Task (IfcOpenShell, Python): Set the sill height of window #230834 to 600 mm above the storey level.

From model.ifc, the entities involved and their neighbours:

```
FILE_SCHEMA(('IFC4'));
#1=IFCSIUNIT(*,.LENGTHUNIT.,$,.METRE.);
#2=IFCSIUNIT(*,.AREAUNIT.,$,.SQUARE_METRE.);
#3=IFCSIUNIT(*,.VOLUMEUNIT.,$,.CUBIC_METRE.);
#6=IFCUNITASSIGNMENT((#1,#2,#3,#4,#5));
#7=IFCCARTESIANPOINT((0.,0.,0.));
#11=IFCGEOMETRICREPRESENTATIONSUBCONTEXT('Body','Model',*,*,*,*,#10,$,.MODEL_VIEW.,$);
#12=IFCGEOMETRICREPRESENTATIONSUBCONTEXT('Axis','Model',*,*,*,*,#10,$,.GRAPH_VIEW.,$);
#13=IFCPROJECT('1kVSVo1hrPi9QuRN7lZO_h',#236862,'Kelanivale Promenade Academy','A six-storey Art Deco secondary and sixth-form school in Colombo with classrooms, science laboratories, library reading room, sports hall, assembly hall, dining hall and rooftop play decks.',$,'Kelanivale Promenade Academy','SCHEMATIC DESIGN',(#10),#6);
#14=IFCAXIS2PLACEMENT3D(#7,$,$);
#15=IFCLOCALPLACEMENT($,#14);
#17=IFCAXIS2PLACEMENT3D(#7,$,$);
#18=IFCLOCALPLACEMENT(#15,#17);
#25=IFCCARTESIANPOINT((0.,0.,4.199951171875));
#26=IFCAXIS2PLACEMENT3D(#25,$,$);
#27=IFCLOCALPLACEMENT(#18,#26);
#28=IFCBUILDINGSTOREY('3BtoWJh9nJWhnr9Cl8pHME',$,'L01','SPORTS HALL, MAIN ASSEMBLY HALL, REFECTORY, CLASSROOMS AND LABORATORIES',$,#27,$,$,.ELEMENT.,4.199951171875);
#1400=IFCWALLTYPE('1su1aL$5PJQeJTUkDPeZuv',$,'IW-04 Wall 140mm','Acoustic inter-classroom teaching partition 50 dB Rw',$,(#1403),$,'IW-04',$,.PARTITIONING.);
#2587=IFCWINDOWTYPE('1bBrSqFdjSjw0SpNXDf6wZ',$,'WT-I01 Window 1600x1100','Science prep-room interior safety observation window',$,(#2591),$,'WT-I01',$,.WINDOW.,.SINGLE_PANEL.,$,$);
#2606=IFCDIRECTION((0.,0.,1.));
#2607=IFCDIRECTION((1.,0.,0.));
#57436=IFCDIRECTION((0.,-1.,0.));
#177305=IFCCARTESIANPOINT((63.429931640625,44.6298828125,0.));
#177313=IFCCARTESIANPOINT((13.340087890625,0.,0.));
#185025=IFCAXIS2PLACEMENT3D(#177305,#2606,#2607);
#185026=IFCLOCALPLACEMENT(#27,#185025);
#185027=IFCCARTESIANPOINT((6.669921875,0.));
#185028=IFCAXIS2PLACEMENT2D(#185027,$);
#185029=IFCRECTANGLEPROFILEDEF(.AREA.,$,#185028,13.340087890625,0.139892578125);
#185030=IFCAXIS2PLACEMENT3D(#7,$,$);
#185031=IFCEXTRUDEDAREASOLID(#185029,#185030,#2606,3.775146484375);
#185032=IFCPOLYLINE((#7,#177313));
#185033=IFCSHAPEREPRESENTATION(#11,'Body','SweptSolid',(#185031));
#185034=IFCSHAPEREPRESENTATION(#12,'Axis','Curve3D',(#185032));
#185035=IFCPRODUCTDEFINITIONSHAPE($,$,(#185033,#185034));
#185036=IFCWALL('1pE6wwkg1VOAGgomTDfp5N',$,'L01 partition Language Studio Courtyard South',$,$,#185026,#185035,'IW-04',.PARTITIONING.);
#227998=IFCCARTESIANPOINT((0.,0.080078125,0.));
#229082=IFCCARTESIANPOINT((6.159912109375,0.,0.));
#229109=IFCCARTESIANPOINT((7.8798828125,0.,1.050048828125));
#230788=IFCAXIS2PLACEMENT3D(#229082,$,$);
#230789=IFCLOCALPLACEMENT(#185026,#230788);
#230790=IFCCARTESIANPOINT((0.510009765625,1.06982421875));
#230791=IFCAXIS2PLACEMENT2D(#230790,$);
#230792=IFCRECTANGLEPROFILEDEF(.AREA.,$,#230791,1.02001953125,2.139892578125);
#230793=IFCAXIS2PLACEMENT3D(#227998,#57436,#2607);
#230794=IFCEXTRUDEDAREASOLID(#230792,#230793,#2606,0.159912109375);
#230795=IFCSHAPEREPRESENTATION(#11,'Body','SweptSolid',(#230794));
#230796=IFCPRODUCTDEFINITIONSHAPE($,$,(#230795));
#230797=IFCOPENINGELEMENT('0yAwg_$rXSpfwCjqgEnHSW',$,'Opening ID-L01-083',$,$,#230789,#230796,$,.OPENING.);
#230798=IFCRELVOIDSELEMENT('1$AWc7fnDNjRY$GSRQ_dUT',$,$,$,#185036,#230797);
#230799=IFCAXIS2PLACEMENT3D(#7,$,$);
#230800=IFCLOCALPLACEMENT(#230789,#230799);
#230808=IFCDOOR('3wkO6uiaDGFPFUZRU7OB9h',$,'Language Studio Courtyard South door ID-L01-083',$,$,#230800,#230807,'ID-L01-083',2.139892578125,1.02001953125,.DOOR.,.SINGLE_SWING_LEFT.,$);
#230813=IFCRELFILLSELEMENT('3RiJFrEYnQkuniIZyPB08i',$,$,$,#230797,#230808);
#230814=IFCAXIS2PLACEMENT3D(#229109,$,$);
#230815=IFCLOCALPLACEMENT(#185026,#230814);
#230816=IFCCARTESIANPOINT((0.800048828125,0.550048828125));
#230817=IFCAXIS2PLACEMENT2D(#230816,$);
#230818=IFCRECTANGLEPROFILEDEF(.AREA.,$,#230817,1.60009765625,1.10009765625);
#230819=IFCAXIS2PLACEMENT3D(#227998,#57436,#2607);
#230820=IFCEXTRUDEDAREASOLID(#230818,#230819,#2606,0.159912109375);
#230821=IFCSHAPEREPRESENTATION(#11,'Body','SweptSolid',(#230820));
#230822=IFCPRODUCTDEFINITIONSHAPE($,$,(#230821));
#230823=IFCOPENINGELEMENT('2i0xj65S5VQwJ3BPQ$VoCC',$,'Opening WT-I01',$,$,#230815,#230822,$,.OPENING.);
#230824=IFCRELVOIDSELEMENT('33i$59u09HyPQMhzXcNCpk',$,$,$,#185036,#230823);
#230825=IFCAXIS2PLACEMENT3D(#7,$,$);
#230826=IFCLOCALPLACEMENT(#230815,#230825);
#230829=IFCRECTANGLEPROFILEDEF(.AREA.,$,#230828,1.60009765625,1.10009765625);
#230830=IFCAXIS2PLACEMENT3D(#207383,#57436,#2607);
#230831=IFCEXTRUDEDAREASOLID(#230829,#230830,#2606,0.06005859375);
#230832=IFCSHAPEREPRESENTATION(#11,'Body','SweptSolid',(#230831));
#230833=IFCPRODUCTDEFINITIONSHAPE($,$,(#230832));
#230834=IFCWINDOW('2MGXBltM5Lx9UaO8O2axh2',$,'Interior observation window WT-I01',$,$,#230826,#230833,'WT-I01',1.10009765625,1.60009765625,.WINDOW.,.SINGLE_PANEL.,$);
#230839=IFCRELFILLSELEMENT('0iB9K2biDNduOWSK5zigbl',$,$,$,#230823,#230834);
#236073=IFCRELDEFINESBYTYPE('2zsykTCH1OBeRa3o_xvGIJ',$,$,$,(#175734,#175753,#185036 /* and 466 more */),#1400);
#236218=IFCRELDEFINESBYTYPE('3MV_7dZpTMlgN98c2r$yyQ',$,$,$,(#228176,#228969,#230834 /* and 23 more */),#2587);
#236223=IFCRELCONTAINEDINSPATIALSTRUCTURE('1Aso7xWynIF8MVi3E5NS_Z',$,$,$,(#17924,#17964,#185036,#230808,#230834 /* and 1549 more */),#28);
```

```python
import numpy as np
import ifcopenshell
import ifcopenshell.api.geometry
import ifcopenshell.geom
import ifcopenshell.util.element
import ifcopenshell.util.placement
import ifcopenshell.util.shape
import ifcopenshell.util.unit

model = ifcopenshell.open("model.ifc")
unit_scale = ifcopenshell.util.unit.calculate_unit_scale(model)

window = model.by_id(230834)
opening = window.FillsVoids[0].RelatingOpeningElement
storey = ifcopenshell.util.element.get_container(window, ifc_class="IfcBuildingStorey")
level = ifcopenshell.util.placement.get_local_placement(storey.ObjectPlacement)[2, 3]

# The opening's origin need not be at the sill, so measure its lowest point.
shape = ifcopenshell.geom.create_shape(ifcopenshell.geom.settings(), opening)
bottom = ifcopenshell.util.shape.get_shape_bottom_elevation(shape, shape.geometry) / unit_scale
dz = level + 0.6 / unit_scale - bottom

shift = np.array([0.0, 0.0, dz])
# The window is placed relative to its opening, so it follows when the opening moves.
matrix = ifcopenshell.util.placement.get_local_placement(opening.ObjectPlacement)
matrix[:3, 3] += shift
ifcopenshell.api.geometry.edit_object_placement(
    model, product=opening, matrix=matrix, is_si=False, should_transform_children=True
)

print(f"moved by {dz * unit_scale:+.3f} m")

model.write("model_rev.ifc")
```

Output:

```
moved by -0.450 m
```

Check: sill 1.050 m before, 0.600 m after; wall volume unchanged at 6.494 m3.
